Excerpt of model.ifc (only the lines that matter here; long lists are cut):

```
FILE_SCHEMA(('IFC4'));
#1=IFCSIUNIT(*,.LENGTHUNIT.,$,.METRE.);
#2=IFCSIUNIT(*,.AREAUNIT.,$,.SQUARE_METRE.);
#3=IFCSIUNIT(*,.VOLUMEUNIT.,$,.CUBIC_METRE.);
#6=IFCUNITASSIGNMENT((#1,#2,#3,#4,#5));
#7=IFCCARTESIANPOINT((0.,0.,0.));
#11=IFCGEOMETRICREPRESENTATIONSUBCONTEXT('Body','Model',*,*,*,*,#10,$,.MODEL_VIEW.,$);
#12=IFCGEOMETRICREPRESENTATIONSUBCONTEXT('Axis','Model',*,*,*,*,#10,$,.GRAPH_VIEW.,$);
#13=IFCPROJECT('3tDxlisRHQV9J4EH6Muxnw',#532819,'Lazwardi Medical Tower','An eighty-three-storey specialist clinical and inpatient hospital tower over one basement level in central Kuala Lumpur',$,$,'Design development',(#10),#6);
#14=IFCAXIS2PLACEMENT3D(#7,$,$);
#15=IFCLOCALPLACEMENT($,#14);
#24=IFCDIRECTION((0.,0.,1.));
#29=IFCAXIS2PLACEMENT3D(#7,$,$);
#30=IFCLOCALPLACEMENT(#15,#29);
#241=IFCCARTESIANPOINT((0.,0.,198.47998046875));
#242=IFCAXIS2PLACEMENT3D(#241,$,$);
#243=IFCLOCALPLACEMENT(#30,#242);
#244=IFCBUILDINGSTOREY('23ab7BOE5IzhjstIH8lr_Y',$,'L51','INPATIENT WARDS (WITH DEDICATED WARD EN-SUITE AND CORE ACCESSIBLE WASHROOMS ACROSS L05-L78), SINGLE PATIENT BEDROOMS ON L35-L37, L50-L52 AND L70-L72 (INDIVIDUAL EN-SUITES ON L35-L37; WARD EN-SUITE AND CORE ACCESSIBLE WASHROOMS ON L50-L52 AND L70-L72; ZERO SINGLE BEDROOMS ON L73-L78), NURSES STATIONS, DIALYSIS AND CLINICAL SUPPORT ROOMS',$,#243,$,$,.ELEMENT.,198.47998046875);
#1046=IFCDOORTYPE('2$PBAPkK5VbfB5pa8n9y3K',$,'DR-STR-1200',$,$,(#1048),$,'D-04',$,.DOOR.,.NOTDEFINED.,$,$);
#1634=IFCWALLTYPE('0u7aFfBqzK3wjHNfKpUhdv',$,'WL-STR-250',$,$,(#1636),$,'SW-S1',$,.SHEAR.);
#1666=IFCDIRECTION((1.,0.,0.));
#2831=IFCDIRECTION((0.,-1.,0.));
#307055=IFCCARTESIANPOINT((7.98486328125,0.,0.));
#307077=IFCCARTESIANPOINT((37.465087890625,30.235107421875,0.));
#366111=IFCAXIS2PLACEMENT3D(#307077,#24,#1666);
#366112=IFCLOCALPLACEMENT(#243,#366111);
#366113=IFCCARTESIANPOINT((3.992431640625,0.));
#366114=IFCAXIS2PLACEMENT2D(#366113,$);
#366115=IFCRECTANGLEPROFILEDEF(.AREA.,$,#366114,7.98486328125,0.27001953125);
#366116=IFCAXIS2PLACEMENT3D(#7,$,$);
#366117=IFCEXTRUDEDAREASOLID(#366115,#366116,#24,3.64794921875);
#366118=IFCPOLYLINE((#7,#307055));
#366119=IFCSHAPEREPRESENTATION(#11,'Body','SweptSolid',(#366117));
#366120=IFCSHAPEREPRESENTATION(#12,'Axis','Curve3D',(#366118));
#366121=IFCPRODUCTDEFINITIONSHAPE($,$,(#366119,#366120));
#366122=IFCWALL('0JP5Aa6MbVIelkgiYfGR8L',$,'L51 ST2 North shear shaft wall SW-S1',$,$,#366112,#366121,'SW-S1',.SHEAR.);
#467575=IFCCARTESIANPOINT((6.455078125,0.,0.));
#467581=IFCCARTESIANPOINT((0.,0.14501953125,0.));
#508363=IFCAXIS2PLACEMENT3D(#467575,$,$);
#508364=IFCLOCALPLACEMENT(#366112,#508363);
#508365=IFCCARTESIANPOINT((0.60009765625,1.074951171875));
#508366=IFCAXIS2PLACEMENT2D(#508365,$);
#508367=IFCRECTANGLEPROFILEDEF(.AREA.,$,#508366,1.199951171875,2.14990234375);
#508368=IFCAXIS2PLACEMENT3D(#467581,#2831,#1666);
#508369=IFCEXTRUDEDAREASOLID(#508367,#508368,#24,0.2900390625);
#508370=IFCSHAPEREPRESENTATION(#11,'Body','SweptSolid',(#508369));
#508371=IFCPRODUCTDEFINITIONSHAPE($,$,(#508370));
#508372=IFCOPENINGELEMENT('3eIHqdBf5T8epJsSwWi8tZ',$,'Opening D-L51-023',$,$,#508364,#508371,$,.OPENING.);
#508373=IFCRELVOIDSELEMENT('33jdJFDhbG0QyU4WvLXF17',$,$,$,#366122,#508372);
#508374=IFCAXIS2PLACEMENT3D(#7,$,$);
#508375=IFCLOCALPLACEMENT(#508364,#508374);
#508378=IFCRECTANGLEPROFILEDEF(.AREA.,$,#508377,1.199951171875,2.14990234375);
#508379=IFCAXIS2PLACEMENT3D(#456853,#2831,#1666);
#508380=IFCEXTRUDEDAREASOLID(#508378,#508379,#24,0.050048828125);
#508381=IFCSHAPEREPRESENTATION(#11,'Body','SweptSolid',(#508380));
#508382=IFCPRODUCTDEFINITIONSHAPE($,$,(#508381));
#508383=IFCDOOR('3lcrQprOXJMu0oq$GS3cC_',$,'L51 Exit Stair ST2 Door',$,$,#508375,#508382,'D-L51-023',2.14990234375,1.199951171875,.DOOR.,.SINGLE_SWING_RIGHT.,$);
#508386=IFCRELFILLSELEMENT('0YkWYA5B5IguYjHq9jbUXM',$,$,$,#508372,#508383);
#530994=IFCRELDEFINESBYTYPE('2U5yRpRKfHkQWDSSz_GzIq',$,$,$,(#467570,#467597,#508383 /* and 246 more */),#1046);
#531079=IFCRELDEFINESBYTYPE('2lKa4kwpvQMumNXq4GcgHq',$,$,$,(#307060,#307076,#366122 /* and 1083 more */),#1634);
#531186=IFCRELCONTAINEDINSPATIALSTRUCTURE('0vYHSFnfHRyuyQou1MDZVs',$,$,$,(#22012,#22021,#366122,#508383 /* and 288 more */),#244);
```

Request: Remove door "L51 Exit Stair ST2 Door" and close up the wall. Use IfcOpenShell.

```python
import ifcopenshell
import ifcopenshell.api.feature
import ifcopenshell.api.root
import ifcopenshell.geom
import ifcopenshell.util.shape

model = ifcopenshell.open("model.ifc")
settings = ifcopenshell.geom.settings()


def volume(element):
    """Net volume in cubic metres, openings subtracted."""
    shape = ifcopenshell.geom.create_shape(settings, element)
    return ifcopenshell.util.shape.get_volume(shape.geometry)


door = model.by_guid("3lcrQprOXJMu0oq$GS3cC_")
opening = door.FillsVoids[0].RelatingOpeningElement
wall = opening.VoidsElements[0].RelatingBuildingElement
before = volume(wall)

ifcopenshell.api.root.remove_product(model, product=door)
ifcopenshell.api.feature.remove_feature(model, feature=opening)

after = volume(wall)

print(f"wall volume {before:.3f} -> {after:.3f} m3")

model.write("model_updated.ifc")
```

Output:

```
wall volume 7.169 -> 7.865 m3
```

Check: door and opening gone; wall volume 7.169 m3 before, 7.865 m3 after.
